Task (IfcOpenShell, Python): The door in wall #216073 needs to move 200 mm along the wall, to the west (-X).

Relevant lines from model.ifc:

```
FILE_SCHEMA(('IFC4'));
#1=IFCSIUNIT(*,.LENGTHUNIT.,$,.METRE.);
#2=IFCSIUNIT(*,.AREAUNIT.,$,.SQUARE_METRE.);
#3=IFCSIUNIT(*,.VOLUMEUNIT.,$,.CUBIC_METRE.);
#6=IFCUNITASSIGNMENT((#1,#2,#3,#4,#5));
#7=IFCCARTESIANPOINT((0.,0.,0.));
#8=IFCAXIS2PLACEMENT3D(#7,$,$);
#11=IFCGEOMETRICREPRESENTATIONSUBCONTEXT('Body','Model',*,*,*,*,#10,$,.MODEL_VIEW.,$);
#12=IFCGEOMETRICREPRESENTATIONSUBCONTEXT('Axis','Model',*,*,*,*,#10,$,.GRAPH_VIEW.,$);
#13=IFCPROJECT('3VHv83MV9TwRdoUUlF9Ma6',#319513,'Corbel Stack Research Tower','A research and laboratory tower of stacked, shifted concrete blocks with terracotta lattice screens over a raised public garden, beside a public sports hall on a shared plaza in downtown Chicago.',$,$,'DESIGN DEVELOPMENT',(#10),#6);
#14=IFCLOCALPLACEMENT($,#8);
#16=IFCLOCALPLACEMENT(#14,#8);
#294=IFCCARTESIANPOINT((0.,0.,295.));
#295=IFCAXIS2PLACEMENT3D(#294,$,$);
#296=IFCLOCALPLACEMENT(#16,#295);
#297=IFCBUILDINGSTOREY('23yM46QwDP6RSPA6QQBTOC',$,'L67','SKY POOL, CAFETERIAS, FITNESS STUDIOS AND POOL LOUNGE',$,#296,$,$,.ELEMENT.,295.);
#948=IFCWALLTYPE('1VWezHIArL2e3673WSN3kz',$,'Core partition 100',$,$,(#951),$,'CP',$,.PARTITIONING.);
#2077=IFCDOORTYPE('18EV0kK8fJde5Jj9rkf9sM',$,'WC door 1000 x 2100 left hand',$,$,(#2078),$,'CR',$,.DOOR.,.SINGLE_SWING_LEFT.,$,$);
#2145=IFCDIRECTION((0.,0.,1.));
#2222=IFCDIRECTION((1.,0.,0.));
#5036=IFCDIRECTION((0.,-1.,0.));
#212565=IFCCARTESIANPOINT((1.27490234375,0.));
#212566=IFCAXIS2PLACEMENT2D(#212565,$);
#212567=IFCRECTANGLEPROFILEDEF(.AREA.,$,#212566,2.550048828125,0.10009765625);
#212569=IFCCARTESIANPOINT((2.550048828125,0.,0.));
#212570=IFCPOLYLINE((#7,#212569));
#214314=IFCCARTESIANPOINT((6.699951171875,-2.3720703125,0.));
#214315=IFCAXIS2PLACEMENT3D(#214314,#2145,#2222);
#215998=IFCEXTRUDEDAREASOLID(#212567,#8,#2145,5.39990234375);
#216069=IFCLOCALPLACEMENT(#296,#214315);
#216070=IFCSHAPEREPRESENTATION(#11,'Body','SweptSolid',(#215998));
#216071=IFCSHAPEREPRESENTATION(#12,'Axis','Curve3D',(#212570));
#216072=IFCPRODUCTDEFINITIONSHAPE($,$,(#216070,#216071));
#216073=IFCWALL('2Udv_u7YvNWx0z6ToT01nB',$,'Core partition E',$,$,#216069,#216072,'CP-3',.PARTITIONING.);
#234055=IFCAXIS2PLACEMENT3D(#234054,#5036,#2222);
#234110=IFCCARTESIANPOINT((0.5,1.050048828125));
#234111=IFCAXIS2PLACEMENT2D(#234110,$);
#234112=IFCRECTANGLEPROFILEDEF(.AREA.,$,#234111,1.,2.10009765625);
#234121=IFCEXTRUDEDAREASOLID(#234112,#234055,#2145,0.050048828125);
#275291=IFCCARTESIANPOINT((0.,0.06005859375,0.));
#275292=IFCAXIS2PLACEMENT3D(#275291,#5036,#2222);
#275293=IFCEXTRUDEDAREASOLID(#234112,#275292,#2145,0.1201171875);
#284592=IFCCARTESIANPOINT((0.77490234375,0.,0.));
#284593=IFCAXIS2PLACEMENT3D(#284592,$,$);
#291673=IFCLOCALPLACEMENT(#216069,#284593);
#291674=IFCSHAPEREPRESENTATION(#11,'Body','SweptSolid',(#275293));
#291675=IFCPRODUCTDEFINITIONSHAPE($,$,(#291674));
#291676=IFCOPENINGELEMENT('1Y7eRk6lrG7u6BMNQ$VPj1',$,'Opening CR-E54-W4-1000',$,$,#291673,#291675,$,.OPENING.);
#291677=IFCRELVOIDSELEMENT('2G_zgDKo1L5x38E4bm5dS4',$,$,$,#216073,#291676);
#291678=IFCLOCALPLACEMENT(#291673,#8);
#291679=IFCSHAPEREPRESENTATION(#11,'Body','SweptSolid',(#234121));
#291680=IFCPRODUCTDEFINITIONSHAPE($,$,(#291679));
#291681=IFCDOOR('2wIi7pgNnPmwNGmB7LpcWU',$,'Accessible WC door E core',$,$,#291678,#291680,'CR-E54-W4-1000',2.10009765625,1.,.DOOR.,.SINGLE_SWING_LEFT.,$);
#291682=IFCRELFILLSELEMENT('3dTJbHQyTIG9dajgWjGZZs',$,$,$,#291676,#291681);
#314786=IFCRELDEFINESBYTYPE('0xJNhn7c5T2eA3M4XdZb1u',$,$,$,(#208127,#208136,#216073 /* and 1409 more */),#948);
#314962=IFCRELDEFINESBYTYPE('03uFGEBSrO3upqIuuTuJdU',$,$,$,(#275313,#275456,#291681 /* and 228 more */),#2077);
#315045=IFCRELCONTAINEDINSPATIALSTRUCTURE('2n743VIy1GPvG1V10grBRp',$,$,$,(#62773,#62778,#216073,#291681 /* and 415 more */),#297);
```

```python
import ifcopenshell
import ifcopenshell.api.geometry
import ifcopenshell.util.placement
import ifcopenshell.util.unit

model = ifcopenshell.open("model.ifc")
unit_scale = ifcopenshell.util.unit.calculate_unit_scale(model)

door = model.by_guid("2wIi7pgNnPmwNGmB7LpcWU")
opening = door.FillsVoids[0].RelatingOpeningElement
wall = opening.VoidsElements[0].RelatingBuildingElement

wall_matrix = ifcopenshell.util.placement.get_local_placement(wall.ObjectPlacement)
shift = wall_matrix[:3, 0] * -0.2 / unit_scale
before = ifcopenshell.util.placement.get_local_placement(door.ObjectPlacement)[:3, 3].copy()

# The door is placed relative to its opening, so it follows when the opening moves.
matrix = ifcopenshell.util.placement.get_local_placement(opening.ObjectPlacement)
matrix[:3, 3] += shift
ifcopenshell.api.geometry.edit_object_placement(
    model, product=opening, matrix=matrix, is_si=False, should_transform_children=True
)

after = ifcopenshell.util.placement.get_local_placement(door.ObjectPlacement)[:3, 3]
print("door moved by", (after - before).round(3) + 0.0)

model.write("model_v2.ifc")
```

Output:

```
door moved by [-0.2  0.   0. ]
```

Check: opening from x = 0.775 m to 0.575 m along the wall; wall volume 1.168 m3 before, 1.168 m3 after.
